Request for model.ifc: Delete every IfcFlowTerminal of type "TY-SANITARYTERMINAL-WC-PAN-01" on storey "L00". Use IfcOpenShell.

First a look at what the model holds.

```python
import ifcopenshell
import ifcopenshell.util.element

model = ifcopenshell.open("model.ifc")
print(model.schema)
storey = next(s for s in model.by_type("IfcBuildingStorey") if s.Name == "L00")
terminals = [e for e in ifcopenshell.util.element.get_decomposition(storey) if e.is_a("IfcFlowTerminal")]
seen = {}
for e in terminals:
    element_type = ifcopenshell.util.element.get_type(e)
    name = element_type.Name if element_type not in (None, e) else None
    seen[name] = seen.get(name, 0) + 1
for name, count in sorted(seen.items(), key=str):
    print(count, "x", name)
```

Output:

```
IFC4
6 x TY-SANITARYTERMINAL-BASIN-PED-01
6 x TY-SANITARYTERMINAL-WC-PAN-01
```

```python
import ifcopenshell
import ifcopenshell.api.root
import ifcopenshell.util.element

model = ifcopenshell.open("model.ifc")

storey = next(s for s in model.by_type("IfcBuildingStorey") if s.Name == "L00")
terminals = [e for e in ifcopenshell.util.element.get_decomposition(storey) if e.is_a("IfcFlowTerminal")]
targets = [e for e in terminals if (t := ifcopenshell.util.element.get_type(e)) not in (None, e) and t.Name == "TY-SANITARYTERMINAL-WC-PAN-01"]

for e in targets:
    ifcopenshell.api.root.remove_product(model, product=e)
print(len(targets), "removed")

model.write("model_rev.ifc")
```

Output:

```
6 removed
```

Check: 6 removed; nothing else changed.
